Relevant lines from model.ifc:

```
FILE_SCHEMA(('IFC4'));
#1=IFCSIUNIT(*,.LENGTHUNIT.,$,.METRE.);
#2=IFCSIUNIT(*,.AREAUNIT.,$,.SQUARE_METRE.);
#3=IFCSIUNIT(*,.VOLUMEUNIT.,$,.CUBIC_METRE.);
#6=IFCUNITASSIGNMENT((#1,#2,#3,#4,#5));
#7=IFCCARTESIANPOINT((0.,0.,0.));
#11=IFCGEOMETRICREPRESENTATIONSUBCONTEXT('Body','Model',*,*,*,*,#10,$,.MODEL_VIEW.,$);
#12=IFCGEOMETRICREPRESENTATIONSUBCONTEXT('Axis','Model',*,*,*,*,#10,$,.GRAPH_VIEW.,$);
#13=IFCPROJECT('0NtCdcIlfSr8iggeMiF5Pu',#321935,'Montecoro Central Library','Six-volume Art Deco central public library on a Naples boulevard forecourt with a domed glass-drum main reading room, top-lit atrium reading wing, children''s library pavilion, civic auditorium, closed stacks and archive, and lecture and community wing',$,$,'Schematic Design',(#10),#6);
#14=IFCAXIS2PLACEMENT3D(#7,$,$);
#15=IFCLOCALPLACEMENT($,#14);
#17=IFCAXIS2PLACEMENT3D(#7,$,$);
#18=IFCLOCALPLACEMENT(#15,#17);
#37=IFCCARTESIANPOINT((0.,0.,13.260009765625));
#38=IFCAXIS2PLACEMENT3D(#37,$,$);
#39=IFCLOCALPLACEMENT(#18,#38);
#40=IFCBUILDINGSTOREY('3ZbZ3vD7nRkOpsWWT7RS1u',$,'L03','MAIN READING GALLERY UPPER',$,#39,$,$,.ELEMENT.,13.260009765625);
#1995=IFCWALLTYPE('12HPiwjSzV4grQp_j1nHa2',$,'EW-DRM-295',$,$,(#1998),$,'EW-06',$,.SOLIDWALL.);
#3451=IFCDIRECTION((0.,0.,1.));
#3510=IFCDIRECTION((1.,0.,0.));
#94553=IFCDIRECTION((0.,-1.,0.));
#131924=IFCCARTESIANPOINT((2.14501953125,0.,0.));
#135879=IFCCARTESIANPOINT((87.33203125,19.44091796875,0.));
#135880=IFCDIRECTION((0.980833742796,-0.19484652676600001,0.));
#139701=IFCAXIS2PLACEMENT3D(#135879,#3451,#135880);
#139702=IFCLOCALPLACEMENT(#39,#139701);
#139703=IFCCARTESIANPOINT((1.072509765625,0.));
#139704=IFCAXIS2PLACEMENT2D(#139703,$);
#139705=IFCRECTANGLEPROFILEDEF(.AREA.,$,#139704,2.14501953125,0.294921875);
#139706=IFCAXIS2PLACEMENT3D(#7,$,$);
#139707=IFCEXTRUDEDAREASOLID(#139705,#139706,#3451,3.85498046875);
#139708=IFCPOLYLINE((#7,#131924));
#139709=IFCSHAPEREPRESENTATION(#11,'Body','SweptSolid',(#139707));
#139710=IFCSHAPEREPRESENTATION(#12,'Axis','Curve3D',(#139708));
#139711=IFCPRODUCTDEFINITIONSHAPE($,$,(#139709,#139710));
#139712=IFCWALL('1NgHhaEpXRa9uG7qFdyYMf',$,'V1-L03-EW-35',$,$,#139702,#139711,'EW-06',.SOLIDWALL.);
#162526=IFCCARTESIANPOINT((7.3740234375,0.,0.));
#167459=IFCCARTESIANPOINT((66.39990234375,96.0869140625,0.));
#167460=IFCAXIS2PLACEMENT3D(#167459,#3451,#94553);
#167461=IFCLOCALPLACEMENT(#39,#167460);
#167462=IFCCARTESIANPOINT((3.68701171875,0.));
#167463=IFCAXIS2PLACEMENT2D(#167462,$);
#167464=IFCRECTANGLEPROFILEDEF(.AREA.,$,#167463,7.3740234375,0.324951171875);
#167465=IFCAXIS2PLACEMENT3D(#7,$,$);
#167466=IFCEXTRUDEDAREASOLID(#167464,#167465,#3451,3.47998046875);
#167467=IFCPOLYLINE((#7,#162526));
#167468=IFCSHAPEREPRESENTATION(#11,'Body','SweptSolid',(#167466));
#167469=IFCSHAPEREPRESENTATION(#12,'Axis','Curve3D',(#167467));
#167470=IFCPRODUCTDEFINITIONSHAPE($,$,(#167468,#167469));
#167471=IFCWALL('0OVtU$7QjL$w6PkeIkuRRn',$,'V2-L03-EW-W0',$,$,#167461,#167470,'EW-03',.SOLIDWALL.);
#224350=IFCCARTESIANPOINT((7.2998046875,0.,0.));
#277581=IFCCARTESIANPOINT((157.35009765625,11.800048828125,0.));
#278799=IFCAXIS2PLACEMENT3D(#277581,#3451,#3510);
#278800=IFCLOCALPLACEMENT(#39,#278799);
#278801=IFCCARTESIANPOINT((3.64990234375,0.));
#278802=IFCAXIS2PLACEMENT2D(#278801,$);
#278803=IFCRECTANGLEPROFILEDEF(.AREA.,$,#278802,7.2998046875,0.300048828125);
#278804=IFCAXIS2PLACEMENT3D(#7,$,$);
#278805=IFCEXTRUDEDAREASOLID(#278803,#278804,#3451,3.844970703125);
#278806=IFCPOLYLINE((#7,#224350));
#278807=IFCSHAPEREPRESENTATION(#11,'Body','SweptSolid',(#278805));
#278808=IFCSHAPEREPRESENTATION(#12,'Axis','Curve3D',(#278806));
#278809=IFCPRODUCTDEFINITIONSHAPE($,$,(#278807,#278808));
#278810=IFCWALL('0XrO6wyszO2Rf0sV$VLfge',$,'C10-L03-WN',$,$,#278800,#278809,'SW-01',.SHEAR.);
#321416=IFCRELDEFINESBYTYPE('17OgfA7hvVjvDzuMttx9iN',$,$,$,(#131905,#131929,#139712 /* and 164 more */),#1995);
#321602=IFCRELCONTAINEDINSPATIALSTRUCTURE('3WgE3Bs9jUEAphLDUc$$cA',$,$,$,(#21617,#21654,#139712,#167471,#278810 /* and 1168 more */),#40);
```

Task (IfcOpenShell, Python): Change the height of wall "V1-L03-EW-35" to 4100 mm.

```python
import ifcopenshell
import ifcopenshell.geom
import ifcopenshell.util.representation
import ifcopenshell.util.shape

model = ifcopenshell.open("model.ifc")
settings = ifcopenshell.geom.settings()


def volume(element):
    """Net volume in cubic metres, openings subtracted."""
    shape = ifcopenshell.geom.create_shape(settings, element)
    return ifcopenshell.util.shape.get_volume(shape.geometry)


wall = model.by_guid("1NgHhaEpXRa9uG7qFdyYMf")
before = volume(wall)

body = ifcopenshell.util.representation.get_representation(wall, "Model", "Body")
solid = body.Items[0]
old_height = solid.Depth
solid.Depth = 4.1
after = volume(wall)

print(f"height {old_height:g} -> {solid.Depth:g}, volume {before:.3f} -> {after:.3f} m3")

model.write("model_v2.ifc")
```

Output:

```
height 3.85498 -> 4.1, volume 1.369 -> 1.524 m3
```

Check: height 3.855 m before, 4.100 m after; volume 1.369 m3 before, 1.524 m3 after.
